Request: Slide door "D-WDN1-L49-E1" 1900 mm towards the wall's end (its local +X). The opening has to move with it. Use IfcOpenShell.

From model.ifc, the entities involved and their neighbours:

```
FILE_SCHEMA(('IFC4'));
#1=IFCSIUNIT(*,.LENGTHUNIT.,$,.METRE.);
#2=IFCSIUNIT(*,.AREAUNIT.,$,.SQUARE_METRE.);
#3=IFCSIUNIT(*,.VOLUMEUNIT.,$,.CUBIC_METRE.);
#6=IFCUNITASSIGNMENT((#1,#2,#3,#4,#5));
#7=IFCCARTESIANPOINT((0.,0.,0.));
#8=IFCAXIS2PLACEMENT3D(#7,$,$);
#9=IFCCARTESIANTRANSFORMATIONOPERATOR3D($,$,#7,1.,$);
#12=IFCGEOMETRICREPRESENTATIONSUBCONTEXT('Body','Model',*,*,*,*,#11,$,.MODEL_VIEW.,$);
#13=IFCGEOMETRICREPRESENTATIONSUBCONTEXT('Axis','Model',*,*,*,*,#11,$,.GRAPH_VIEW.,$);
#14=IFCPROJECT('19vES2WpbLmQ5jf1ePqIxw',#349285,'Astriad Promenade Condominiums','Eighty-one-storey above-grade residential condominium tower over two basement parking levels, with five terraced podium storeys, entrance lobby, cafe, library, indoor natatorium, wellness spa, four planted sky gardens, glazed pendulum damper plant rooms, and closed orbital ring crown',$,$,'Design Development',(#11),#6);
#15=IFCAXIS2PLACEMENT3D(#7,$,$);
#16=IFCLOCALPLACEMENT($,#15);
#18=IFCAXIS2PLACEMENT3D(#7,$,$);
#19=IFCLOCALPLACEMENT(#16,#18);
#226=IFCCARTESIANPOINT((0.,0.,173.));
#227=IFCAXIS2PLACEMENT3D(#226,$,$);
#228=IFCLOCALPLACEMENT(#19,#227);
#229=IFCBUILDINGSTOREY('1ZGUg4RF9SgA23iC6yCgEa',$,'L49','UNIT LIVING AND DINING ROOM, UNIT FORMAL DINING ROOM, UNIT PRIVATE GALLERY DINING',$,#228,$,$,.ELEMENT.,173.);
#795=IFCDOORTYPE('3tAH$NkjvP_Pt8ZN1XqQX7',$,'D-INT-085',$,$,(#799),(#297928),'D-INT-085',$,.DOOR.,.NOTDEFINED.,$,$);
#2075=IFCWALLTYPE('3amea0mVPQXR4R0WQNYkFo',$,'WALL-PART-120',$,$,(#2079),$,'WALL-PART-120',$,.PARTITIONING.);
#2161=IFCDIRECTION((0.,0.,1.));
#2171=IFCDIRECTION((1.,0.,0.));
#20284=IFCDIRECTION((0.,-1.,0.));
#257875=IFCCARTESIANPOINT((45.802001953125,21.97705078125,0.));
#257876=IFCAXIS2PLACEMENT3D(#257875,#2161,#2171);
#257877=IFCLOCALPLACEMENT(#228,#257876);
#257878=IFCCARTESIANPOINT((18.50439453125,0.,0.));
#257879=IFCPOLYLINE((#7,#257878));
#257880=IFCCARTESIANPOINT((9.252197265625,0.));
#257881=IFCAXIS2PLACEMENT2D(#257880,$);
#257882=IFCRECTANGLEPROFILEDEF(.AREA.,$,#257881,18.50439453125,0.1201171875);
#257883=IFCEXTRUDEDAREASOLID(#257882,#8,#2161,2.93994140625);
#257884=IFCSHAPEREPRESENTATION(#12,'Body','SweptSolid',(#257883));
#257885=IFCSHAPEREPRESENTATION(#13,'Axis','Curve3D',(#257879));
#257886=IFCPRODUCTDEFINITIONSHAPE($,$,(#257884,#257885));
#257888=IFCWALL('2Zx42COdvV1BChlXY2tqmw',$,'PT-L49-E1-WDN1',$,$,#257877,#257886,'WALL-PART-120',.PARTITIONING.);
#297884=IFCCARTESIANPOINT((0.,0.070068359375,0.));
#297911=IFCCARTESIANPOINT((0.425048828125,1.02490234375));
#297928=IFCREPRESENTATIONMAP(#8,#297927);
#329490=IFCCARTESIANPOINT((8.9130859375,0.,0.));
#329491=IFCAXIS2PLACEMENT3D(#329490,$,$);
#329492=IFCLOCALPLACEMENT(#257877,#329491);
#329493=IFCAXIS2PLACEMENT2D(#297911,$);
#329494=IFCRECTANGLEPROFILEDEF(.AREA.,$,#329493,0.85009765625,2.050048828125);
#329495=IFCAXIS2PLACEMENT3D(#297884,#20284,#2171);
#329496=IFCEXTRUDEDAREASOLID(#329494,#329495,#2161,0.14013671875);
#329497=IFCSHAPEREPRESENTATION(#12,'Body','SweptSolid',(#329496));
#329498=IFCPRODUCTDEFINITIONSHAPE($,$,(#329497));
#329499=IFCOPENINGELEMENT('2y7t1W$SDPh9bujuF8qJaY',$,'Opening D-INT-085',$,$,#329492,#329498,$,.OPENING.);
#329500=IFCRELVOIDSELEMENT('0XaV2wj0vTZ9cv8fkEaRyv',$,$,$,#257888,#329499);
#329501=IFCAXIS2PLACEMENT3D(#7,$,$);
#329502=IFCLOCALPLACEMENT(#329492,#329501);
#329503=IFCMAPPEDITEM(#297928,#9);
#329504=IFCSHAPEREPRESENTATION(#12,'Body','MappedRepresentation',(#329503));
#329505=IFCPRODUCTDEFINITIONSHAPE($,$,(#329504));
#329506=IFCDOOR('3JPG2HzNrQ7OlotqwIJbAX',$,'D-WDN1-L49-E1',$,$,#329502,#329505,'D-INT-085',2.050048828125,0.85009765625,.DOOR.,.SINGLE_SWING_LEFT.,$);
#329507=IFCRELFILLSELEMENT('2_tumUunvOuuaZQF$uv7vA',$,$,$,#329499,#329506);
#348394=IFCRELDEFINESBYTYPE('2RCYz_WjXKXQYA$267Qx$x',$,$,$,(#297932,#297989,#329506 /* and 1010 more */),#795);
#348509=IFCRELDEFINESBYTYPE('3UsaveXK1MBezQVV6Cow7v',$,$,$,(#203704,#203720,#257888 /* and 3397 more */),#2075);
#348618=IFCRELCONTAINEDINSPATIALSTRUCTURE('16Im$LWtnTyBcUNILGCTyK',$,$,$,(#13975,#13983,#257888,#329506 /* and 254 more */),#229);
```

```python
import ifcopenshell
import ifcopenshell.api.geometry
import ifcopenshell.util.placement
import ifcopenshell.util.unit

model = ifcopenshell.open("model.ifc")
unit_scale = ifcopenshell.util.unit.calculate_unit_scale(model)

door = model.by_guid("3JPG2HzNrQ7OlotqwIJbAX")
opening = door.FillsVoids[0].RelatingOpeningElement
wall = opening.VoidsElements[0].RelatingBuildingElement

wall_matrix = ifcopenshell.util.placement.get_local_placement(wall.ObjectPlacement)
shift = wall_matrix[:3, 0] * 1.9 / unit_scale
before = ifcopenshell.util.placement.get_local_placement(door.ObjectPlacement)[:3, 3].copy()

# The door is placed relative to its opening, so it follows when the opening moves.
matrix = ifcopenshell.util.placement.get_local_placement(opening.ObjectPlacement)
matrix[:3, 3] += shift
ifcopenshell.api.geometry.edit_object_placement(
    model, product=opening, matrix=matrix, is_si=False, should_transform_children=True
)

after = ifcopenshell.util.placement.get_local_placement(door.ObjectPlacement)[:3, 3]
print("door moved by", (after - before).round(3) + 0.0)

model.write("model_rev.ifc")
```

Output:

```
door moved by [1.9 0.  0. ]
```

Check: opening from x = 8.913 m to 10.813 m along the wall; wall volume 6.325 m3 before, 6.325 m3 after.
